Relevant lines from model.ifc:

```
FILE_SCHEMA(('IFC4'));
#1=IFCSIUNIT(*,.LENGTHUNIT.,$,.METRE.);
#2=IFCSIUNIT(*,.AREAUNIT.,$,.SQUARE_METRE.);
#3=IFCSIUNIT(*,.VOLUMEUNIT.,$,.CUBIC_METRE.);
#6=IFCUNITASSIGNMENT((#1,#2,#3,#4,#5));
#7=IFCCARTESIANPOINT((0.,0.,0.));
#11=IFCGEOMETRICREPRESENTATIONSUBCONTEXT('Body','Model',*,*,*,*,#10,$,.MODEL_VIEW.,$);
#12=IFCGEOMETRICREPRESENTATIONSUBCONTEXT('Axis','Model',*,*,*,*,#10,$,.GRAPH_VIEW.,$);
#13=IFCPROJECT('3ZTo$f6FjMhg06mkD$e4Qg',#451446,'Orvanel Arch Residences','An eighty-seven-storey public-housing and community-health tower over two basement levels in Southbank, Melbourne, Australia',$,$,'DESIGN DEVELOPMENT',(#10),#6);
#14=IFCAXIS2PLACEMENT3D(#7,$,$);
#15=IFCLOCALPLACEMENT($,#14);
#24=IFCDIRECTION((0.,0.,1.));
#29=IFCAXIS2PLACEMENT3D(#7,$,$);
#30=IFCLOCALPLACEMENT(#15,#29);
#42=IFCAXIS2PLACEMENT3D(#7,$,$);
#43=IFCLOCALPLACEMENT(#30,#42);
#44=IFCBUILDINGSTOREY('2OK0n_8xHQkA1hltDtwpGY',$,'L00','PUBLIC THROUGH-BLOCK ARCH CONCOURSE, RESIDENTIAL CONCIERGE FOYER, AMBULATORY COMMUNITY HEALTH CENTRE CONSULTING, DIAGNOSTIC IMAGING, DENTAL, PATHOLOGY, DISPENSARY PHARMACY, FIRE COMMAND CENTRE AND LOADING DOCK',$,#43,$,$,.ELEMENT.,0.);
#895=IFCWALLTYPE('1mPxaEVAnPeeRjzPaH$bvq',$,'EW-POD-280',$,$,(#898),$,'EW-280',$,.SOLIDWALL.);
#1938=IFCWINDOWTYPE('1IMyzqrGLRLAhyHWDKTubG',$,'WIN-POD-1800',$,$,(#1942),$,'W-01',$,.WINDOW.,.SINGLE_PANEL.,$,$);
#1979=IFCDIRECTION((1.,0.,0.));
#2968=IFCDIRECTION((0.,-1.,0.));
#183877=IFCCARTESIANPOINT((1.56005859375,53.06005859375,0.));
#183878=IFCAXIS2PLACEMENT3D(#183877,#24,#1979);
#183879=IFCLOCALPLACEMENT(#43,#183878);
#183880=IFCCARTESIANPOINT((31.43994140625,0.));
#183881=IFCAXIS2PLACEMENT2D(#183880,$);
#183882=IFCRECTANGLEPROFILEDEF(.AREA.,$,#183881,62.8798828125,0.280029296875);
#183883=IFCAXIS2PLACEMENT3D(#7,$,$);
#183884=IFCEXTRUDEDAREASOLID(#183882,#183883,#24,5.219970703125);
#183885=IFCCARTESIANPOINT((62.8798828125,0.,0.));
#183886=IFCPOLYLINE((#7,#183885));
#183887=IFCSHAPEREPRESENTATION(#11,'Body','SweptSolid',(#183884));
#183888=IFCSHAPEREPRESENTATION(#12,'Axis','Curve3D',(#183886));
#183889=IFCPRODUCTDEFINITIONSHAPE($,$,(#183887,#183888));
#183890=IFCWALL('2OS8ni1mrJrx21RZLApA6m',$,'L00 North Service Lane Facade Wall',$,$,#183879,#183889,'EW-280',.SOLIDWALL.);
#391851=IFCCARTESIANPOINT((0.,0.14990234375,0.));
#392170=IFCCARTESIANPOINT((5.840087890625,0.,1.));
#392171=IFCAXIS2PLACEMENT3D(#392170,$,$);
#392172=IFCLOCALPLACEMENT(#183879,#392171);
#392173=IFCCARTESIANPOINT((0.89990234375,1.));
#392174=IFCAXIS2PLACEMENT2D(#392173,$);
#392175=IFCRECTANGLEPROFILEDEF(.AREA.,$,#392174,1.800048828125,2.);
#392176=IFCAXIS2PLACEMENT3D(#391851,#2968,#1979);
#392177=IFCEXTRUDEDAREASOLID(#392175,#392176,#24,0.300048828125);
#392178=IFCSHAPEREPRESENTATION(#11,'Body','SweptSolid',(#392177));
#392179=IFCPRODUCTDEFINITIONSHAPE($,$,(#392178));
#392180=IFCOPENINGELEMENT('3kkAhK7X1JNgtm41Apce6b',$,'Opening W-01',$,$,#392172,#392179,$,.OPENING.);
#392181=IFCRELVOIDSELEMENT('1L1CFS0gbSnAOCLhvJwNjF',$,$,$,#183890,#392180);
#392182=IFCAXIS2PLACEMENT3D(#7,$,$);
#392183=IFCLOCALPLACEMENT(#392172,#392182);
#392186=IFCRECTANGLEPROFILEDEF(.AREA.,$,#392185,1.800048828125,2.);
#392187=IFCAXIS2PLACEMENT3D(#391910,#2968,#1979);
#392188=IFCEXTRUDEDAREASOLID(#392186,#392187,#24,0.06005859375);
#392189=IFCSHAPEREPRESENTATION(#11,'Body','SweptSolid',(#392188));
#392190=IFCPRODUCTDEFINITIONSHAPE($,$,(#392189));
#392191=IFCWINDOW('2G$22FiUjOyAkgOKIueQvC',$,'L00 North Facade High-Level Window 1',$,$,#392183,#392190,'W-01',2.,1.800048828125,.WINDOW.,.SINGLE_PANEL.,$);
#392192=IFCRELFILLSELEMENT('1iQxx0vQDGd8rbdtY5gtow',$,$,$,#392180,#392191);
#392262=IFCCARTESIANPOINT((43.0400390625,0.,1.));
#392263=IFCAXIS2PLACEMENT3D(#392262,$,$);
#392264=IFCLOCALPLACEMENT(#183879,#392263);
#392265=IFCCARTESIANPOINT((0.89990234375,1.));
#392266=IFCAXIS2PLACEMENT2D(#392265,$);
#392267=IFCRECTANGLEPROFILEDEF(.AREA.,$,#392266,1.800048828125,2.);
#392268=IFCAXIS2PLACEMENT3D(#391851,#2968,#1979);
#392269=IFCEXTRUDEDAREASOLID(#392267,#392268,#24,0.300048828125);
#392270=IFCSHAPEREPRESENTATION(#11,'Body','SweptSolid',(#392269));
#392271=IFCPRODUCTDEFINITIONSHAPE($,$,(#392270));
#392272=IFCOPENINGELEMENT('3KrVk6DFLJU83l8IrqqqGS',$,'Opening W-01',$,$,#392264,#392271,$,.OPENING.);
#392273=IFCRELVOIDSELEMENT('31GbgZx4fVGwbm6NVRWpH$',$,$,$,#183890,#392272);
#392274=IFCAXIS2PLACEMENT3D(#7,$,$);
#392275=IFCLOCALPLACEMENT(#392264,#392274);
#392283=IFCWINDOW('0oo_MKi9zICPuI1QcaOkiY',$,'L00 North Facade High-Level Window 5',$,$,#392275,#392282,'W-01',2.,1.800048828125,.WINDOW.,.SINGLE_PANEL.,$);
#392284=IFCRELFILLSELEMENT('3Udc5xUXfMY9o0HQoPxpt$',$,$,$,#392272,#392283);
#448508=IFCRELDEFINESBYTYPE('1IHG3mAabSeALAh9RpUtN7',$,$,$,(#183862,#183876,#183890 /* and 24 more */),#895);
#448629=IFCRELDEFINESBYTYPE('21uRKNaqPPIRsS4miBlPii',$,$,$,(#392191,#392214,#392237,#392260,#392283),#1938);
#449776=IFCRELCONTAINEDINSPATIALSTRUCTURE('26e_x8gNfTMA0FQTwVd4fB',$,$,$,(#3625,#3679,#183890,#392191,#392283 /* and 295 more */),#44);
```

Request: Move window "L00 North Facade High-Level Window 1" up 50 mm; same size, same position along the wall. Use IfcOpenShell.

```python
import numpy as np
import ifcopenshell
import ifcopenshell.api.geometry
import ifcopenshell.util.placement
import ifcopenshell.util.unit

model = ifcopenshell.open("model.ifc")
unit_scale = ifcopenshell.util.unit.calculate_unit_scale(model)

window = model.by_id(392191)
opening = window.FillsVoids[0].RelatingOpeningElement
dz = 0.05 / unit_scale

shift = np.array([0.0, 0.0, dz])
# The window is placed relative to its opening, so it follows when the opening moves.
matrix = ifcopenshell.util.placement.get_local_placement(opening.ObjectPlacement)
matrix[:3, 3] += shift
ifcopenshell.api.geometry.edit_object_placement(
    model, product=opening, matrix=matrix, is_si=False, should_transform_children=True
)

print(f"moved by {dz * unit_scale:+.3f} m")

model.write("model_v2.ifc")
```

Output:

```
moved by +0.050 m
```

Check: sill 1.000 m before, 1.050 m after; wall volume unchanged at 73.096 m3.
